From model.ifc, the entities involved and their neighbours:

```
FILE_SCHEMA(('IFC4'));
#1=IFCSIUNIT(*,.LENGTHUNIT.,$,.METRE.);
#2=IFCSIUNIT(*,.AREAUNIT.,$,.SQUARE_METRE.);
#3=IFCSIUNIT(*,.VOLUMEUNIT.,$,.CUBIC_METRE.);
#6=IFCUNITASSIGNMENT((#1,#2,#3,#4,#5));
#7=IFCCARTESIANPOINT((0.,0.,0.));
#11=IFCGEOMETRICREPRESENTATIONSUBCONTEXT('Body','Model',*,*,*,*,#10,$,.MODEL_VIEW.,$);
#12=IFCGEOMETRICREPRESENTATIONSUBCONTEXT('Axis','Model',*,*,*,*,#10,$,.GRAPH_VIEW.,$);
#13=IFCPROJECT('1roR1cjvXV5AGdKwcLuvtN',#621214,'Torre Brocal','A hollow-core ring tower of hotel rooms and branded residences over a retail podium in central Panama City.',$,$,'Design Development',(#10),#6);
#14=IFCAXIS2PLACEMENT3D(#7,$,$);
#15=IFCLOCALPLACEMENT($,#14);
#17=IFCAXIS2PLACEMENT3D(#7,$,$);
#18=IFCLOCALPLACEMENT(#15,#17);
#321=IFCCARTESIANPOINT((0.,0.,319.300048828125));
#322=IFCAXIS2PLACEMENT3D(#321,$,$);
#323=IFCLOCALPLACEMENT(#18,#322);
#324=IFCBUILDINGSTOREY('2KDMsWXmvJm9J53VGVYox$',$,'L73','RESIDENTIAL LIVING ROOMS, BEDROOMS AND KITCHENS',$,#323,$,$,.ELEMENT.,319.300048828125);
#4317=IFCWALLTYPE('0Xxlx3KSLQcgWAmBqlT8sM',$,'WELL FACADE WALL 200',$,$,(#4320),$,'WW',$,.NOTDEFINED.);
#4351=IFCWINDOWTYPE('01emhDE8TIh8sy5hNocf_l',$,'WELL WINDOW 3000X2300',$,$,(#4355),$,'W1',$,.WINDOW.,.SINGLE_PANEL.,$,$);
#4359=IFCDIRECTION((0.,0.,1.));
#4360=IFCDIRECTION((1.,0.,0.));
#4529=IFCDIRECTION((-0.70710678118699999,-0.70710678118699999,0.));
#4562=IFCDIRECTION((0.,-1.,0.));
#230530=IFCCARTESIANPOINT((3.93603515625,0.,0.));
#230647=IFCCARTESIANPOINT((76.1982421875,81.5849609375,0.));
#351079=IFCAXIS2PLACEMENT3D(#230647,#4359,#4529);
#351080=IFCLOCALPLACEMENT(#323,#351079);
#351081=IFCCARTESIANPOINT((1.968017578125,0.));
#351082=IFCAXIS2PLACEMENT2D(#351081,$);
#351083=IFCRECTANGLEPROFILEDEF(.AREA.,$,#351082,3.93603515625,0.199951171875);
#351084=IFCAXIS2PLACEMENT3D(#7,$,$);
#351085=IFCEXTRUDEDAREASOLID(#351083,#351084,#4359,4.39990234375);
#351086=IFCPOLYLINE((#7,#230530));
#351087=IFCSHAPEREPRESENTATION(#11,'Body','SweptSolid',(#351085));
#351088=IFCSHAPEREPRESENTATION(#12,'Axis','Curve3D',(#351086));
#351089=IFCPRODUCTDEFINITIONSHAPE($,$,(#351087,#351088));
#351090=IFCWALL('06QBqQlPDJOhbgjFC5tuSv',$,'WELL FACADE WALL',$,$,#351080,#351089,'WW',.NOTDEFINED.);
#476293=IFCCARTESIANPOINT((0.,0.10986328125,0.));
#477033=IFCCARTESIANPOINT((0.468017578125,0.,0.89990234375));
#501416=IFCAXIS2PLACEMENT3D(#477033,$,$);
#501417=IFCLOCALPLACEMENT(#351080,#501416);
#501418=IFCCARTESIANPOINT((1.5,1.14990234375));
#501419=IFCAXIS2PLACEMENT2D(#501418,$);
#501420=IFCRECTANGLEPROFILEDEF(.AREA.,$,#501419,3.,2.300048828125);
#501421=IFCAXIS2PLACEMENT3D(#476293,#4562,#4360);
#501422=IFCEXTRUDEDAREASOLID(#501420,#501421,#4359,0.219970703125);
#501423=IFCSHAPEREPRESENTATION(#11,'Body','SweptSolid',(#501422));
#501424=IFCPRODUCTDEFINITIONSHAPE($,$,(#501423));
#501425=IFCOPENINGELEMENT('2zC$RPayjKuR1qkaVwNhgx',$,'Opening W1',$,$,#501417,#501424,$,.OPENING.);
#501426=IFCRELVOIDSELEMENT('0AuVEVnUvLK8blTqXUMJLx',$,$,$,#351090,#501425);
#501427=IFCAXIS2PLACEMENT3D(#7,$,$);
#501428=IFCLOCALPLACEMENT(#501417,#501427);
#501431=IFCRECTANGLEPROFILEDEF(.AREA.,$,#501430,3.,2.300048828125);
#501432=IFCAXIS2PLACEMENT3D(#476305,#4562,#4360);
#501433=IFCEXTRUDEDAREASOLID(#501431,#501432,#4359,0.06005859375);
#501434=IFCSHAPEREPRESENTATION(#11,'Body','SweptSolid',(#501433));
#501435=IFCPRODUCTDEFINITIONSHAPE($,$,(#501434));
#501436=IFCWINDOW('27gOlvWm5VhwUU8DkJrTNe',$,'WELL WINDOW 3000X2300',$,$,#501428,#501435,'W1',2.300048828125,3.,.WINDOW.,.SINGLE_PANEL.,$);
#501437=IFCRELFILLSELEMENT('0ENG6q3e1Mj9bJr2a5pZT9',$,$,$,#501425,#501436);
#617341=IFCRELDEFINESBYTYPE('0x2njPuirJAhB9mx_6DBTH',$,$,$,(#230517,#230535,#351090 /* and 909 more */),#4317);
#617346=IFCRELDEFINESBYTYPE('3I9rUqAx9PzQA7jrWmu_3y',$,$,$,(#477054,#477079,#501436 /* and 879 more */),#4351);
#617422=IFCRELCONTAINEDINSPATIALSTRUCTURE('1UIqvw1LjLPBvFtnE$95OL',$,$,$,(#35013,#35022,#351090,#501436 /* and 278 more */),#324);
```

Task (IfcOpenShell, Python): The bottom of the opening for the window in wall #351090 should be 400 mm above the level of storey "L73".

```python
import numpy as np
import ifcopenshell
import ifcopenshell.api.geometry
import ifcopenshell.geom
import ifcopenshell.util.element
import ifcopenshell.util.placement
import ifcopenshell.util.shape
import ifcopenshell.util.unit

model = ifcopenshell.open("model.ifc")
unit_scale = ifcopenshell.util.unit.calculate_unit_scale(model)

window = model.by_id(501436)
opening = window.FillsVoids[0].RelatingOpeningElement
storey = ifcopenshell.util.element.get_container(window, ifc_class="IfcBuildingStorey")
level = ifcopenshell.util.placement.get_local_placement(storey.ObjectPlacement)[2, 3]

# The opening's origin need not be at the sill, so measure its lowest point.
shape = ifcopenshell.geom.create_shape(ifcopenshell.geom.settings(), opening)
bottom = ifcopenshell.util.shape.get_shape_bottom_elevation(shape, shape.geometry) / unit_scale
dz = level + 0.4 / unit_scale - bottom

shift = np.array([0.0, 0.0, dz])
# The window is placed relative to its opening, so it follows when the opening moves.
matrix = ifcopenshell.util.placement.get_local_placement(opening.ObjectPlacement)
matrix[:3, 3] += shift
ifcopenshell.api.geometry.edit_object_placement(
    model, product=opening, matrix=matrix, is_si=False, should_transform_children=True
)

print(f"moved by {dz * unit_scale:+.3f} m")

model.write("model_edited.ifc")
```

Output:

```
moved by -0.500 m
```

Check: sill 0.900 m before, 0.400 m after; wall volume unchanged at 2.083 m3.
